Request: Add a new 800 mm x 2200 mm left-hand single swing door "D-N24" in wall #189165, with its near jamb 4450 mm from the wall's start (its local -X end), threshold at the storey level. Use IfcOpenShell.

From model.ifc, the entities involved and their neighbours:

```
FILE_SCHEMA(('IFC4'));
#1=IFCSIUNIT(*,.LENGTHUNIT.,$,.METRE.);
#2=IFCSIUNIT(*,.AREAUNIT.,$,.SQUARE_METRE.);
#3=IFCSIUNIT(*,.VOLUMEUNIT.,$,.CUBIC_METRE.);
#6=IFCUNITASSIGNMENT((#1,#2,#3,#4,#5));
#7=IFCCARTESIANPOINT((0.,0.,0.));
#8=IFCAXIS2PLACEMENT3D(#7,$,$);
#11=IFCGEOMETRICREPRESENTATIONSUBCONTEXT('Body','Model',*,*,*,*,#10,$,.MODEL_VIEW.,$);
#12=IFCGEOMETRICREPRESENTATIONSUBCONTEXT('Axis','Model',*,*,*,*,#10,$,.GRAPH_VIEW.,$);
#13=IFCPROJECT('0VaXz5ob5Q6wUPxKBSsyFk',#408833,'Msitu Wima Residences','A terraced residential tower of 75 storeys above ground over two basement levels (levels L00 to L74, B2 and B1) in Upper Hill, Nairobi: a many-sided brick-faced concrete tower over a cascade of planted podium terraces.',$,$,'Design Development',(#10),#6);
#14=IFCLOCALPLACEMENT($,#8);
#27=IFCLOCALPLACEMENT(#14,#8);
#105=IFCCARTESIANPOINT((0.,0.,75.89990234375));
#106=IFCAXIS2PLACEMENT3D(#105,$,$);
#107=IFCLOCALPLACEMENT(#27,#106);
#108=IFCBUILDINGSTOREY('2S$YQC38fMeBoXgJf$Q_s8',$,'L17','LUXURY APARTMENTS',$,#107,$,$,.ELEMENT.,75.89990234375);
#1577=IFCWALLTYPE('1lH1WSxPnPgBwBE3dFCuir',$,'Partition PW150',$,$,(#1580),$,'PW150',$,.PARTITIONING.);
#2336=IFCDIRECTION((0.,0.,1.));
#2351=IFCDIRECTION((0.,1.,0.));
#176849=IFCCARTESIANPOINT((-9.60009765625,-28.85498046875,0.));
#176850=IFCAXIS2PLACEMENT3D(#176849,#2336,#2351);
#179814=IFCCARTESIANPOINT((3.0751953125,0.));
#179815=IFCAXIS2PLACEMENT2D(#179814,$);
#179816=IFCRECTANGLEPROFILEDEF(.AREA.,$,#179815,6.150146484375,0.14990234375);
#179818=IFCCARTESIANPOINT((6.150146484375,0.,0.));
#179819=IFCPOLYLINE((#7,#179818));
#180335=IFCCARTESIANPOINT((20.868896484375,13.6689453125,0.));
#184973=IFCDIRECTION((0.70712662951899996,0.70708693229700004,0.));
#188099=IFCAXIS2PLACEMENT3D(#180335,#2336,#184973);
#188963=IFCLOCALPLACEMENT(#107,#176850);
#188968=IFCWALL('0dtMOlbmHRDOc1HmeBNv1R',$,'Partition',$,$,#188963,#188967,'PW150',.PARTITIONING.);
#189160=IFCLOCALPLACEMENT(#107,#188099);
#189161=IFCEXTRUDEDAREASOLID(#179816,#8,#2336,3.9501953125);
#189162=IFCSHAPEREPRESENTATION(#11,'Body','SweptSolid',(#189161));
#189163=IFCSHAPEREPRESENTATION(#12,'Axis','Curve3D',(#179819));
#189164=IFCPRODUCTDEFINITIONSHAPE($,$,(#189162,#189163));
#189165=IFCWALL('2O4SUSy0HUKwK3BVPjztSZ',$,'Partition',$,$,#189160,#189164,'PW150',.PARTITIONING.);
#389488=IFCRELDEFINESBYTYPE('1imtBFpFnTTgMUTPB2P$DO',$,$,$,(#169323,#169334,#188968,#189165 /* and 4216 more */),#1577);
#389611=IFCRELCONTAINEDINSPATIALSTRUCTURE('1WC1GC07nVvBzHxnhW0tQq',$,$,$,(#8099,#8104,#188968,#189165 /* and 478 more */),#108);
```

```python
import numpy as np
import ifcopenshell
import ifcopenshell.api.feature
import ifcopenshell.api.geometry
import ifcopenshell.api.root
import ifcopenshell.api.spatial
import ifcopenshell.geom
import ifcopenshell.util.element
import ifcopenshell.util.placement
import ifcopenshell.util.representation
import ifcopenshell.util.shape
import ifcopenshell.util.unit

model = ifcopenshell.open("model.ifc")
unit_scale = ifcopenshell.util.unit.calculate_unit_scale(model)
settings = ifcopenshell.geom.settings()


def volume(element):
    """Net volume in cubic metres, openings subtracted."""
    shape = ifcopenshell.geom.create_shape(settings, element)
    return ifcopenshell.util.shape.get_volume(shape.geometry)


wall = model.by_id(189165)
storey = ifcopenshell.util.element.get_container(wall, ifc_class="IfcBuildingStorey")
context = ifcopenshell.util.representation.get_context(model, "Model", "Body", "MODEL_VIEW")
before = volume(wall)

width, height, from_end, sill = 0.8, 2.2, 4.45, 0.0  # metres

# The wall runs along its own X axis, and the end named is its -X end.
wall_shape = ifcopenshell.geom.create_shape(settings, wall)
x, y, z = ifcopenshell.util.shape.get_vertices(wall_shape.geometry).T
start = x.min() + from_end
face, thickness = float(y.min()), float(y.max() - y.min())
wall_matrix = ifcopenshell.util.placement.get_local_placement(wall.ObjectPlacement)
level = ifcopenshell.util.placement.get_local_placement(storey.ObjectPlacement)[2, 3]


def in_wall(x, y):
    """Placement at x, y metres in the wall's axes, at sill height."""
    matrix = wall_matrix.copy()
    matrix[:, 3] = wall_matrix @ np.array([x / unit_scale, y / unit_scale, 0.0, 1.0])
    matrix[2, 3] = level + sill / unit_scale
    return matrix


# Opening: a box that overshoots both wall faces by 50 mm.
opening = ifcopenshell.api.root.create_entity(model, ifc_class="IfcOpeningElement", predefined_type="OPENING")
box = ifcopenshell.api.geometry.add_wall_representation(
    model, context=context, length=width, height=height, thickness=thickness + 0.1
)
ifcopenshell.api.geometry.assign_representation(model, product=opening, representation=box)
ifcopenshell.api.geometry.edit_object_placement(model, product=opening, matrix=in_wall(start, face - 0.05), is_si=False)
ifcopenshell.api.feature.add_feature(model, feature=opening, element=wall)

door = ifcopenshell.api.root.create_entity(model, ifc_class="IfcDoor", name="D-N24", predefined_type="DOOR")
door.OverallWidth, door.OverallHeight = width / unit_scale, height / unit_scale
door.OperationType = "SINGLE_SWING_LEFT"
body = ifcopenshell.api.geometry.add_door_representation(
    model,
    context=context,
    overall_width=door.OverallWidth,
    overall_height=door.OverallHeight,
    operation_type="SINGLE_SWING_LEFT",
    lining_properties={"LiningDepth": thickness / unit_scale, "ThresholdDepth": thickness / unit_scale},
)
ifcopenshell.api.geometry.assign_representation(model, product=door, representation=body)
ifcopenshell.api.spatial.assign_container(model, products=[door], relating_structure=storey)
ifcopenshell.api.feature.add_filling(model, opening=opening, element=door)

# The lining spans the wall, so the door starts at the wall face.
ifcopenshell.api.geometry.edit_object_placement(model, product=door, matrix=in_wall(start, face), is_si=False)

after = volume(wall)

print(f"wall volume {before:.3f} -> {after:.3f} m3")

model.write("model_edited.ifc")
```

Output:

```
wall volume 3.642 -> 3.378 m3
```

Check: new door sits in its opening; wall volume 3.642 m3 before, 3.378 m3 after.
